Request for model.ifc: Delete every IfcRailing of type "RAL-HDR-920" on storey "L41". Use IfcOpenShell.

First a look at what the model holds.

```python
import ifcopenshell
import ifcopenshell.util.element

model = ifcopenshell.open("model.ifc")
print(model.schema)
storey = next(s for s in model.by_type("IfcBuildingStorey") if s.Name == "L41")
railings = [e for e in ifcopenshell.util.element.get_decomposition(storey) if e.is_a("IfcRailing")]
seen = {}
for e in railings:
    element_type = ifcopenshell.util.element.get_type(e)
    name = element_type.Name if element_type not in (None, e) else None
    seen[name] = seen.get(name, 0) + 1
for name, count in sorted(seen.items(), key=str):
    print(count, "x", name)
```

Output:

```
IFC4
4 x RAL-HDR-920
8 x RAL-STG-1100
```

```python
import ifcopenshell
import ifcopenshell.api.root
import ifcopenshell.util.element

model = ifcopenshell.open("model.ifc")

storey = next(s for s in model.by_type("IfcBuildingStorey") if s.Name == "L41")
railings = [e for e in ifcopenshell.util.element.get_decomposition(storey) if e.is_a("IfcRailing")]
targets = [e for e in railings if (t := ifcopenshell.util.element.get_type(e)) not in (None, e) and t.Name == "RAL-HDR-920"]

for e in targets:
    ifcopenshell.api.root.remove_product(model, product=e)
print(len(targets), "removed")

model.write("model_updated.ifc")
```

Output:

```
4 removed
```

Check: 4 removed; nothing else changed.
